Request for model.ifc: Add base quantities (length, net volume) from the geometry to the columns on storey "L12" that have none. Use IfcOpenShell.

First a look at what the model holds.

```python
import ifcopenshell
import ifcopenshell.util.element
import ifcopenshell.util.unit

model = ifcopenshell.open("model.ifc")
print(model.schema)
for unit_type in ("LENGTHUNIT", "AREAUNIT", "VOLUMEUNIT"):
    print(unit_type, ifcopenshell.util.unit.calculate_unit_scale(model, unit_type))
storey = next(s for s in model.by_type("IfcBuildingStorey") if s.Name == "L12")
columns = [e for e in ifcopenshell.util.element.get_decomposition(storey) if e.is_a("IfcColumn")]
for e in sorted(columns, key=lambda e: e.id()):
    print(e.id(), e.is_a(), e.Name, list(ifcopenshell.util.element.get_psets(e, qtos_only=True)), sep=" | ")
```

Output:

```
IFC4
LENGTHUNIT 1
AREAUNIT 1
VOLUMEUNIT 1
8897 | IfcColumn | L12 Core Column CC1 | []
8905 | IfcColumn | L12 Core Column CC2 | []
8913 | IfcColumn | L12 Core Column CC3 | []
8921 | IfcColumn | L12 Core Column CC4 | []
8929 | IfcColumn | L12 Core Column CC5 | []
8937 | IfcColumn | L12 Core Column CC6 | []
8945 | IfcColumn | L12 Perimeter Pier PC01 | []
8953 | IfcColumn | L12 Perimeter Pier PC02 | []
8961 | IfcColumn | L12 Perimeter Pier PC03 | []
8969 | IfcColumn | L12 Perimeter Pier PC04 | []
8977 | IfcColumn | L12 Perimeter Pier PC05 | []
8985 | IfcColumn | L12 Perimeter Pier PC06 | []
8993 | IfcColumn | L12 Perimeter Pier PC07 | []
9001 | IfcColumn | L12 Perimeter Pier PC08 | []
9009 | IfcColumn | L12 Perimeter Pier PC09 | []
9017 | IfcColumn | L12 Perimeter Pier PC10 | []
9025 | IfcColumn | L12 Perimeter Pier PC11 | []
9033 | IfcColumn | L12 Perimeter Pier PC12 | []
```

```python
import ifcopenshell
import ifcopenshell.api.pset
import ifcopenshell.geom
import ifcopenshell.util.element
import ifcopenshell.util.shape
import ifcopenshell.util.unit

model = ifcopenshell.open("model.ifc")
unit_scale = ifcopenshell.util.unit.calculate_unit_scale(model)
volume_scale = ifcopenshell.util.unit.calculate_unit_scale(model, "VOLUMEUNIT")
settings = ifcopenshell.geom.settings()

storey = next(s for s in model.by_type("IfcBuildingStorey") if s.Name == "L12")
columns = [e for e in ifcopenshell.util.element.get_decomposition(storey) if e.is_a("IfcColumn")]

for e in sorted(columns, key=lambda e: e.id()):
    if ifcopenshell.util.element.get_psets(e, qtos_only=True, should_inherit=False):
        continue
    # Geometry comes back in metres, in the element's own axes.
    shape = ifcopenshell.geom.create_shape(settings, e)
    values = {
        "Length": ifcopenshell.util.shape.get_z(shape.geometry) / unit_scale,
        "NetVolume": ifcopenshell.util.shape.get_volume(shape.geometry) / volume_scale,
    }
    qto = ifcopenshell.api.pset.add_qto(model, product=e, name="Qto_ColumnBaseQuantities")
    ifcopenshell.api.pset.edit_qto(model, qto=qto, properties=values)
    print(e.id(), {k: round(v, 3) for k, v in values.items()})

model.write("model_edited.ifc")
```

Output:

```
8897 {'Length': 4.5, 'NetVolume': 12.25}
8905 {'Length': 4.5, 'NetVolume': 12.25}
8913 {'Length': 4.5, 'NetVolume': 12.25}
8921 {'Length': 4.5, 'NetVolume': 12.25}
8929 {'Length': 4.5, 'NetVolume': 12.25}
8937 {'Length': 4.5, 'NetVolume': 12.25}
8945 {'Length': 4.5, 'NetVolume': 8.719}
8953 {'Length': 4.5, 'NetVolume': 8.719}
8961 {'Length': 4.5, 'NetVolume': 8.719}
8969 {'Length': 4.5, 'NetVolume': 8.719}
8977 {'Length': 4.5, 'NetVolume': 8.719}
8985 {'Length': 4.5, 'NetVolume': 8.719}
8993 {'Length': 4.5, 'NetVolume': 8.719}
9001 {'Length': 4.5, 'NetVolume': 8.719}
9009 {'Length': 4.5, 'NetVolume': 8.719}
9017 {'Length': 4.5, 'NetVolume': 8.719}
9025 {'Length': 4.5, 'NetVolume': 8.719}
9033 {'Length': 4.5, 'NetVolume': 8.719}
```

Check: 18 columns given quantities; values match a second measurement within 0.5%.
